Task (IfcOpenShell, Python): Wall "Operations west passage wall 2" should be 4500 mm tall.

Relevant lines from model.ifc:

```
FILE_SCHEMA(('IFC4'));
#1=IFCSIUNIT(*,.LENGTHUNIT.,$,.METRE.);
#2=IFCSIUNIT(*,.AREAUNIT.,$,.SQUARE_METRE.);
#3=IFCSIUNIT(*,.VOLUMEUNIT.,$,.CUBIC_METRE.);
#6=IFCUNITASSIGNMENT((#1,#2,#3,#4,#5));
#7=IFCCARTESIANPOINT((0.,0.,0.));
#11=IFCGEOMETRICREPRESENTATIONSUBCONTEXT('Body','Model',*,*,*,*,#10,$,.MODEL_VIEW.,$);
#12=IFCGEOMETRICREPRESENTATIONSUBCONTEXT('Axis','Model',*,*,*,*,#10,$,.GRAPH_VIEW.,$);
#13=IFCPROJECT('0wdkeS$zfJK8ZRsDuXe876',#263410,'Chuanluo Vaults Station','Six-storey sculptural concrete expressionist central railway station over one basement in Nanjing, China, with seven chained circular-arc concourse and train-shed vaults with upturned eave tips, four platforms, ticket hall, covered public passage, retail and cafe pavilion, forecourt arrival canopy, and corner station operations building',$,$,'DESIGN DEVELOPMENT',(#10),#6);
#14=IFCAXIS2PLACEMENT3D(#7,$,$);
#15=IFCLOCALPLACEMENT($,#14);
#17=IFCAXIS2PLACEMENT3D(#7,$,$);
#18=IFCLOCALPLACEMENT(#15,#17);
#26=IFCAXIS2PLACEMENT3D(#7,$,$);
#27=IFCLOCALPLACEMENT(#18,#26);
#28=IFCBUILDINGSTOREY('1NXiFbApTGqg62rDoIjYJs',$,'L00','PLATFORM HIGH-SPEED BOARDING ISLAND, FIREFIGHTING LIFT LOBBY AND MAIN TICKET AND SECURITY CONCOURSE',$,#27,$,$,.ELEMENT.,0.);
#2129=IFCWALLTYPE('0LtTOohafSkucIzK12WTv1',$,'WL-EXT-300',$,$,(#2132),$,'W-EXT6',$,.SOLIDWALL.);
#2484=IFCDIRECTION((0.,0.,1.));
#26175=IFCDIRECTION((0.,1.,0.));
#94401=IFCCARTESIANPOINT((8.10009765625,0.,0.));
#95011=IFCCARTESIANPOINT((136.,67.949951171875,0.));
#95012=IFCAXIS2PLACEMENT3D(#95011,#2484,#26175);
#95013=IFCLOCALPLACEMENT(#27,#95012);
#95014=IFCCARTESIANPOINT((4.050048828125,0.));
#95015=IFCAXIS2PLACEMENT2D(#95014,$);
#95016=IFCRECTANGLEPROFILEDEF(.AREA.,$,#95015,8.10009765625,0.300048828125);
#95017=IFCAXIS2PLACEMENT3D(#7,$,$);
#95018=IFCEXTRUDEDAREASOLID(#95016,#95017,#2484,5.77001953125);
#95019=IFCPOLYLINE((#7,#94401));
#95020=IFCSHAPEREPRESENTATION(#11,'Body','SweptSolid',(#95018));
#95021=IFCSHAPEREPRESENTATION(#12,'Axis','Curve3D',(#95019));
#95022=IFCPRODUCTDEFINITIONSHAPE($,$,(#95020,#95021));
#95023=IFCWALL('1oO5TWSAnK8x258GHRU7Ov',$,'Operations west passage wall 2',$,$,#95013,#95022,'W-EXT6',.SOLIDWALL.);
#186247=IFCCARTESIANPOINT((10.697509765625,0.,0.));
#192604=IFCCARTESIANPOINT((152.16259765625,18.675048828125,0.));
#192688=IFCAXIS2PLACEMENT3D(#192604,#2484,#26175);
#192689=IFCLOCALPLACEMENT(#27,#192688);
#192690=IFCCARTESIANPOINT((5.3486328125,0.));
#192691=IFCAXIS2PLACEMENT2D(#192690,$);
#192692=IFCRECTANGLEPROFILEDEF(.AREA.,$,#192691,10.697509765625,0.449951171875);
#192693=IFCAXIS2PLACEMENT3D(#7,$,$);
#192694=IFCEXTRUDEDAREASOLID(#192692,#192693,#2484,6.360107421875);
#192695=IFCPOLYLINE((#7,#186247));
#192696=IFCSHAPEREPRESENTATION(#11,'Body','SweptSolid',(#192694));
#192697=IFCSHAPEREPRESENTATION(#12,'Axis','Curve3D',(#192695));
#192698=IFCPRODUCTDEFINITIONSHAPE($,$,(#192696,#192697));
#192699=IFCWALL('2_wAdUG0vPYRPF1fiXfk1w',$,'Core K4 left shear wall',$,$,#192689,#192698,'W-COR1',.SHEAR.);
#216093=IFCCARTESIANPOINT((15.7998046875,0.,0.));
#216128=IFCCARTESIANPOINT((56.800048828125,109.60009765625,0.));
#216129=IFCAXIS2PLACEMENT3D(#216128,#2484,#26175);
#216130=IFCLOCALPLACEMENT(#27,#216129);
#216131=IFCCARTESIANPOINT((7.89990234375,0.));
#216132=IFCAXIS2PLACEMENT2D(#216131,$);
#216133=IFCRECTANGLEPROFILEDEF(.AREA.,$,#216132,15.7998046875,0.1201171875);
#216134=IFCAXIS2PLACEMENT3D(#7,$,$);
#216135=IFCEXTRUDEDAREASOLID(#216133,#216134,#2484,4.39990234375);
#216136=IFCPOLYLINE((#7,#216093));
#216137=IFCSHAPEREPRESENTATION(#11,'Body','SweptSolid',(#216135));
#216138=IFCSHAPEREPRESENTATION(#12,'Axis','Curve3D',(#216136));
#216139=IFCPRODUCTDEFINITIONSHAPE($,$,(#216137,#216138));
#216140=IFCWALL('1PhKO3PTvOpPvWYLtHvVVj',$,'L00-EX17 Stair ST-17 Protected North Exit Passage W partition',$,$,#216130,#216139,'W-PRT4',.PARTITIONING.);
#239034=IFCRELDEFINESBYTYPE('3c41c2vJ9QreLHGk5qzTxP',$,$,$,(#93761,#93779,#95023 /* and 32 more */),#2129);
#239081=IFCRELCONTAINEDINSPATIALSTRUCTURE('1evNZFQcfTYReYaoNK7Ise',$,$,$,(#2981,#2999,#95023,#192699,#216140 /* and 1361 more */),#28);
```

```python
import ifcopenshell
import ifcopenshell.geom
import ifcopenshell.util.representation
import ifcopenshell.util.shape

model = ifcopenshell.open("model.ifc")
settings = ifcopenshell.geom.settings()


def volume(element):
    """Net volume in cubic metres, openings subtracted."""
    shape = ifcopenshell.geom.create_shape(settings, element)
    return ifcopenshell.util.shape.get_volume(shape.geometry)


wall = model.by_guid("1oO5TWSAnK8x258GHRU7Ov")
before = volume(wall)

body = ifcopenshell.util.representation.get_representation(wall, "Model", "Body")
solid = body.Items[0]
old_height = solid.Depth
solid.Depth = 4.5
after = volume(wall)

print(f"height {old_height:g} -> {solid.Depth:g}, volume {before:.3f} -> {after:.3f} m3")

model.write("model_updated.ifc")
```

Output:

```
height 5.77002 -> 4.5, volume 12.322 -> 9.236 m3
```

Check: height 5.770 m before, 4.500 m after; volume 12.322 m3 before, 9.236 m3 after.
